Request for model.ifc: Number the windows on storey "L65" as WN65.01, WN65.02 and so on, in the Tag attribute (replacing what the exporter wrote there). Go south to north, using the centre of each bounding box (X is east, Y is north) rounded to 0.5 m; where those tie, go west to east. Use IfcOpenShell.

First a look at what the model holds.

```python
import ifcopenshell
import ifcopenshell.util.element
import ifcopenshell.util.placement

model = ifcopenshell.open("model.ifc")
print(model.schema)
storey = next(s for s in model.by_type("IfcBuildingStorey") if s.Name == "L65")
windows = [e for e in ifcopenshell.util.element.get_decomposition(storey) if e.is_a("IfcWindow")]
for e in sorted(windows, key=lambda e: e.id()):
    origin = ifcopenshell.util.placement.get_local_placement(e.ObjectPlacement)[:3, 3]
    print(e.id(), e.Tag, e.Name, origin.round(2) + 0.0, sep=" | ")
```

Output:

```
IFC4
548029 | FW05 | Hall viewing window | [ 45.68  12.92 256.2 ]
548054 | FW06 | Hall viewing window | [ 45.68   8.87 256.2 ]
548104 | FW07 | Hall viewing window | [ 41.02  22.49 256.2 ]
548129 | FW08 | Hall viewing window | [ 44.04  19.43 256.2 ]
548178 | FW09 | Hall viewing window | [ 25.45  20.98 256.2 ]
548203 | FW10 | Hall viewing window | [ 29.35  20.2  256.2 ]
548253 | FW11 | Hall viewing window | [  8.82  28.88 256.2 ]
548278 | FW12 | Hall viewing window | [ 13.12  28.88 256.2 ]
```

```python
import ifcopenshell
import ifcopenshell.geom
import ifcopenshell.util.element
import ifcopenshell.util.shape

model = ifcopenshell.open("model.ifc")
settings = ifcopenshell.geom.settings()
settings.set("use-world-coords", True)


def centre(element):
    shape = ifcopenshell.geom.create_shape(settings, element)
    return ifcopenshell.util.shape.get_bbox_centroid(shape.geometry)


storey = next(s for s in model.by_type("IfcBuildingStorey") if s.Name == "L65")
windows = [e for e in ifcopenshell.util.element.get_decomposition(storey) if e.is_a("IfcWindow")]

# Insertion points can sit at a corner or the storey origin, so sort by the geometry (in metres).
centres = {e: centre(e) for e in windows}
windows.sort(key=lambda e: (round(centres[e][1] / 0.5), centres[e][0]))

for i, e in enumerate(windows, start=1):
    number = f"WN65.{i:02d}"
    e.Tag = number
    print(e.id(), number)

model.write("model-out.ifc")
```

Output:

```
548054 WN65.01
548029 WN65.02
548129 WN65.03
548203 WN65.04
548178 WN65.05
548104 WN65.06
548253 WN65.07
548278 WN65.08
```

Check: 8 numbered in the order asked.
